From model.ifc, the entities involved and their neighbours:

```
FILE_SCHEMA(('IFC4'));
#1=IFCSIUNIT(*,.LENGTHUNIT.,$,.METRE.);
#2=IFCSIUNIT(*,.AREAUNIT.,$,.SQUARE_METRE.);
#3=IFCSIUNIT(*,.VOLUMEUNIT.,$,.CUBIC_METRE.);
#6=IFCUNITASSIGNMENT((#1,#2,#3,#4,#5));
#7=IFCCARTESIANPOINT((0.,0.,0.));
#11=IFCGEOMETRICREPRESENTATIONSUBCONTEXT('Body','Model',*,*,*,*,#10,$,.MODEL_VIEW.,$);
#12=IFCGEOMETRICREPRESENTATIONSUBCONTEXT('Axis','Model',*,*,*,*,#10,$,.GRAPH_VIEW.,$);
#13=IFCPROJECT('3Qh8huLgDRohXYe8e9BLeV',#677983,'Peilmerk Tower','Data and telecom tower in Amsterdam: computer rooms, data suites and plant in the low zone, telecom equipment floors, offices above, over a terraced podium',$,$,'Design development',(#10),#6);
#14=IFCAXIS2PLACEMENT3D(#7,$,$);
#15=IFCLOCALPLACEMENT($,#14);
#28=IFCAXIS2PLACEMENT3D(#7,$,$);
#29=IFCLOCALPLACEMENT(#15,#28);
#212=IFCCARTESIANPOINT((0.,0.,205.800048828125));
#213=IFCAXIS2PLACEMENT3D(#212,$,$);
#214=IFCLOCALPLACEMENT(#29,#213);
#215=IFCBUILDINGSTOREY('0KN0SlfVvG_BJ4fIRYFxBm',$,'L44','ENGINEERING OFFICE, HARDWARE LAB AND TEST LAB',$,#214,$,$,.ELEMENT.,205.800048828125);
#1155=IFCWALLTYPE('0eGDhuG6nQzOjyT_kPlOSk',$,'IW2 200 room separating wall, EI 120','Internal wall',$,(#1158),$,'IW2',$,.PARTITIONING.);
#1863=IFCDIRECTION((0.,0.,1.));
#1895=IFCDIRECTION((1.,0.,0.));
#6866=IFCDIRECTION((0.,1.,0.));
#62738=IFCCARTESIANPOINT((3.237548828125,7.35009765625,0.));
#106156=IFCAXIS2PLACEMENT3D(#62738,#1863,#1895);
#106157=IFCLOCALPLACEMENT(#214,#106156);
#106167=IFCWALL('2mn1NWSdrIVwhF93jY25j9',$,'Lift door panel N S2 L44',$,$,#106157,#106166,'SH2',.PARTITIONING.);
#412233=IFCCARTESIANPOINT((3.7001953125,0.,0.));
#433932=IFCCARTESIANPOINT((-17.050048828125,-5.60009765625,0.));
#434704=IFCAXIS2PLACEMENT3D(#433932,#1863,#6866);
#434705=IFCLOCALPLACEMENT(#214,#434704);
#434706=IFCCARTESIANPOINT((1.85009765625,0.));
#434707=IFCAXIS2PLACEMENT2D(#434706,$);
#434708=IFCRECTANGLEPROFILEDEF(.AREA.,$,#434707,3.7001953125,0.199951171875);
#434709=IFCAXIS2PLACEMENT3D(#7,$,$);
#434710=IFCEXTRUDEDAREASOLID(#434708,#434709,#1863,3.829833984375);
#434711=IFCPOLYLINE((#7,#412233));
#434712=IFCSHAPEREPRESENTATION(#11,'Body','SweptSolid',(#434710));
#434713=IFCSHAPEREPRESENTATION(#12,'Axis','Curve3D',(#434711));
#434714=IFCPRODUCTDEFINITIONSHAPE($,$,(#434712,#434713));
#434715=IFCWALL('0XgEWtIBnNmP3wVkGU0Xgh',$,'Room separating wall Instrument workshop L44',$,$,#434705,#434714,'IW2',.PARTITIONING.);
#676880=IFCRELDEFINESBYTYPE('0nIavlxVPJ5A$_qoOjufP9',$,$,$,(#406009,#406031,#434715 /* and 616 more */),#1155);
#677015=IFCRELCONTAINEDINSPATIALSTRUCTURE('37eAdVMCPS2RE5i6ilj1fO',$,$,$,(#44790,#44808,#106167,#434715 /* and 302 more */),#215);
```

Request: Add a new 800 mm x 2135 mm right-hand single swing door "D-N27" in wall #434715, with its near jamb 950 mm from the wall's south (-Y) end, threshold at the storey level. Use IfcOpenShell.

```python
import numpy as np
import ifcopenshell
import ifcopenshell.api.feature
import ifcopenshell.api.geometry
import ifcopenshell.api.root
import ifcopenshell.api.spatial
import ifcopenshell.geom
import ifcopenshell.util.element
import ifcopenshell.util.placement
import ifcopenshell.util.representation
import ifcopenshell.util.shape
import ifcopenshell.util.unit

model = ifcopenshell.open("model.ifc")
unit_scale = ifcopenshell.util.unit.calculate_unit_scale(model)
settings = ifcopenshell.geom.settings()


def volume(element):
    """Net volume in cubic metres, openings subtracted."""
    shape = ifcopenshell.geom.create_shape(settings, element)
    return ifcopenshell.util.shape.get_volume(shape.geometry)


wall = model.by_guid("0XgEWtIBnNmP3wVkGU0Xgh")
storey = ifcopenshell.util.element.get_container(wall, ifc_class="IfcBuildingStorey")
context = ifcopenshell.util.representation.get_context(model, "Model", "Body", "MODEL_VIEW")
before = volume(wall)

width, height, from_end, sill = 0.8, 2.135, 0.95, 0.0  # metres

# The wall runs along its own X axis, and the end named is its -X end.
wall_shape = ifcopenshell.geom.create_shape(settings, wall)
x, y, z = ifcopenshell.util.shape.get_vertices(wall_shape.geometry).T
start = x.min() + from_end
face, thickness = float(y.min()), float(y.max() - y.min())
wall_matrix = ifcopenshell.util.placement.get_local_placement(wall.ObjectPlacement)
level = ifcopenshell.util.placement.get_local_placement(storey.ObjectPlacement)[2, 3]


def in_wall(x, y):
    """Placement at x, y metres in the wall's axes, at sill height."""
    matrix = wall_matrix.copy()
    matrix[:, 3] = wall_matrix @ np.array([x / unit_scale, y / unit_scale, 0.0, 1.0])
    matrix[2, 3] = level + sill / unit_scale
    return matrix


# Opening: a box that overshoots both wall faces by 50 mm.
opening = ifcopenshell.api.root.create_entity(model, ifc_class="IfcOpeningElement", predefined_type="OPENING")
box = ifcopenshell.api.geometry.add_wall_representation(
    model, context=context, length=width, height=height, thickness=thickness + 0.1
)
ifcopenshell.api.geometry.assign_representation(model, product=opening, representation=box)
ifcopenshell.api.geometry.edit_object_placement(model, product=opening, matrix=in_wall(start, face - 0.05), is_si=False)
ifcopenshell.api.feature.add_feature(model, feature=opening, element=wall)

door = ifcopenshell.api.root.create_entity(model, ifc_class="IfcDoor", name="D-N27", predefined_type="DOOR")
door.OverallWidth, door.OverallHeight = width / unit_scale, height / unit_scale
door.OperationType = "SINGLE_SWING_RIGHT"
body = ifcopenshell.api.geometry.add_door_representation(
    model,
    context=context,
    overall_width=door.OverallWidth,
    overall_height=door.OverallHeight,
    operation_type="SINGLE_SWING_RIGHT",
    lining_properties={"LiningDepth": thickness / unit_scale, "ThresholdDepth": thickness / unit_scale},
)
ifcopenshell.api.geometry.assign_representation(model, product=door, representation=body)
ifcopenshell.api.spatial.assign_container(model, products=[door], relating_structure=storey)
ifcopenshell.api.feature.add_filling(model, opening=opening, element=door)

# The lining spans the wall, so the door starts at the wall face.
ifcopenshell.api.geometry.edit_object_placement(model, product=door, matrix=in_wall(start, face), is_si=False)

after = volume(wall)

print(f"wall volume {before:.3f} -> {after:.3f} m3")

model.write("model_updated.ifc")
```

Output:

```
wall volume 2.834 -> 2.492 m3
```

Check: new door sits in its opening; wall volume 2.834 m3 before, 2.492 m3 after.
